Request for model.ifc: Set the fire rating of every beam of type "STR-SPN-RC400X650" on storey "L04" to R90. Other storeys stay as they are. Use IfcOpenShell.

First a look at what the model holds.

```python
import ifcopenshell
import ifcopenshell.util.element

model = ifcopenshell.open("model.ifc")
print(model.schema)
storey = next(s for s in model.by_type("IfcBuildingStorey") if s.Name == "L04")
beams = [e for e in ifcopenshell.util.element.get_decomposition(storey) if e.is_a("IfcBeam")]
seen = {}
for e in beams:
    element_type = ifcopenshell.util.element.get_type(e)
    key = (element_type.Name if element_type != e and element_type else None, ifcopenshell.util.element.get_pset(e, "Pset_BeamCommon", "FireRating"))
    seen[key] = seen.get(key, 0) + 1
for (name, value), count in sorted(seen.items(), key=str):
    print(count, "x", name, "|", value)
```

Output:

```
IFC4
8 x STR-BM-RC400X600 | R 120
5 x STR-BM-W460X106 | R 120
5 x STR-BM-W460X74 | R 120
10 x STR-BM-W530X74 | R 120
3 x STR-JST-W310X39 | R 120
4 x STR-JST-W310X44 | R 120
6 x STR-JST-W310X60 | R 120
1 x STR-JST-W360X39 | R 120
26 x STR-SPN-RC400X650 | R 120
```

```python
import ifcopenshell
import ifcopenshell.api.pset
import ifcopenshell.util.element

model = ifcopenshell.open("model.ifc")

storey = next(s for s in model.by_type("IfcBuildingStorey") if s.Name == "L04")
beams = [e for e in ifcopenshell.util.element.get_decomposition(storey) if e.is_a("IfcBeam")]

count = 0
for e in beams:
    element_type = ifcopenshell.util.element.get_type(e)
    if element_type in (None, e) or element_type.Name != "STR-SPN-RC400X650":
        continue
    # add_pset returns the element's existing set when there is one.
    pset = ifcopenshell.api.pset.add_pset(model, product=e, name="Pset_BeamCommon")
    ifcopenshell.api.pset.edit_pset(model, pset=pset, properties={"FireRating": "R90"})
    count += 1

print(count, "beams updated")

model.write("model-out.ifc")
```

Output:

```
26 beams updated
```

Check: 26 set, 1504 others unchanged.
